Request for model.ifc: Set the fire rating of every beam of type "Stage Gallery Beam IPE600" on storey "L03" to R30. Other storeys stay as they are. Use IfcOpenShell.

First a look at what the model holds.

```python
import ifcopenshell
import ifcopenshell.util.element

model = ifcopenshell.open("model.ifc")
print(model.schema)
storey = next(s for s in model.by_type("IfcBuildingStorey") if s.Name == "L03")
beams = [e for e in ifcopenshell.util.element.get_decomposition(storey) if e.is_a("IfcBeam")]
seen = {}
for e in beams:
    element_type = ifcopenshell.util.element.get_type(e)
    key = (element_type.Name if element_type != e and element_type else None, ifcopenshell.util.element.get_pset(e, "Pset_BeamCommon", "FireRating"))
    seen[key] = seen.get(key, 0) + 1
for (name, value), count in sorted(seen.items(), key=str):
    print(count, "x", name, "|", value)
```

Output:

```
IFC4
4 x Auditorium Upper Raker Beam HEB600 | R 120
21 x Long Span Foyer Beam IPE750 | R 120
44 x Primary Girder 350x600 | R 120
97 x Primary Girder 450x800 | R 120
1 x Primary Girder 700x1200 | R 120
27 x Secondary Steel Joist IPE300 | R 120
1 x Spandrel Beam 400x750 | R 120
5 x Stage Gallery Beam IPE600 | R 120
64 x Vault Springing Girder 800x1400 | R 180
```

```python
import ifcopenshell
import ifcopenshell.api.pset
import ifcopenshell.util.element

model = ifcopenshell.open("model.ifc")

storey = next(s for s in model.by_type("IfcBuildingStorey") if s.Name == "L03")
beams = [e for e in ifcopenshell.util.element.get_decomposition(storey) if e.is_a("IfcBeam")]

count = 0
for e in beams:
    element_type = ifcopenshell.util.element.get_type(e)
    if element_type in (None, e) or element_type.Name != "Stage Gallery Beam IPE600":
        continue
    # add_pset returns the element's existing set when there is one.
    pset = ifcopenshell.api.pset.add_pset(model, product=e, name="Pset_BeamCommon")
    ifcopenshell.api.pset.edit_pset(model, pset=pset, properties={"FireRating": "R30"})
    count += 1

print(count, "beams updated")

model.write("model_edited.ifc")
```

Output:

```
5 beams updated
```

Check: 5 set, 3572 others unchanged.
